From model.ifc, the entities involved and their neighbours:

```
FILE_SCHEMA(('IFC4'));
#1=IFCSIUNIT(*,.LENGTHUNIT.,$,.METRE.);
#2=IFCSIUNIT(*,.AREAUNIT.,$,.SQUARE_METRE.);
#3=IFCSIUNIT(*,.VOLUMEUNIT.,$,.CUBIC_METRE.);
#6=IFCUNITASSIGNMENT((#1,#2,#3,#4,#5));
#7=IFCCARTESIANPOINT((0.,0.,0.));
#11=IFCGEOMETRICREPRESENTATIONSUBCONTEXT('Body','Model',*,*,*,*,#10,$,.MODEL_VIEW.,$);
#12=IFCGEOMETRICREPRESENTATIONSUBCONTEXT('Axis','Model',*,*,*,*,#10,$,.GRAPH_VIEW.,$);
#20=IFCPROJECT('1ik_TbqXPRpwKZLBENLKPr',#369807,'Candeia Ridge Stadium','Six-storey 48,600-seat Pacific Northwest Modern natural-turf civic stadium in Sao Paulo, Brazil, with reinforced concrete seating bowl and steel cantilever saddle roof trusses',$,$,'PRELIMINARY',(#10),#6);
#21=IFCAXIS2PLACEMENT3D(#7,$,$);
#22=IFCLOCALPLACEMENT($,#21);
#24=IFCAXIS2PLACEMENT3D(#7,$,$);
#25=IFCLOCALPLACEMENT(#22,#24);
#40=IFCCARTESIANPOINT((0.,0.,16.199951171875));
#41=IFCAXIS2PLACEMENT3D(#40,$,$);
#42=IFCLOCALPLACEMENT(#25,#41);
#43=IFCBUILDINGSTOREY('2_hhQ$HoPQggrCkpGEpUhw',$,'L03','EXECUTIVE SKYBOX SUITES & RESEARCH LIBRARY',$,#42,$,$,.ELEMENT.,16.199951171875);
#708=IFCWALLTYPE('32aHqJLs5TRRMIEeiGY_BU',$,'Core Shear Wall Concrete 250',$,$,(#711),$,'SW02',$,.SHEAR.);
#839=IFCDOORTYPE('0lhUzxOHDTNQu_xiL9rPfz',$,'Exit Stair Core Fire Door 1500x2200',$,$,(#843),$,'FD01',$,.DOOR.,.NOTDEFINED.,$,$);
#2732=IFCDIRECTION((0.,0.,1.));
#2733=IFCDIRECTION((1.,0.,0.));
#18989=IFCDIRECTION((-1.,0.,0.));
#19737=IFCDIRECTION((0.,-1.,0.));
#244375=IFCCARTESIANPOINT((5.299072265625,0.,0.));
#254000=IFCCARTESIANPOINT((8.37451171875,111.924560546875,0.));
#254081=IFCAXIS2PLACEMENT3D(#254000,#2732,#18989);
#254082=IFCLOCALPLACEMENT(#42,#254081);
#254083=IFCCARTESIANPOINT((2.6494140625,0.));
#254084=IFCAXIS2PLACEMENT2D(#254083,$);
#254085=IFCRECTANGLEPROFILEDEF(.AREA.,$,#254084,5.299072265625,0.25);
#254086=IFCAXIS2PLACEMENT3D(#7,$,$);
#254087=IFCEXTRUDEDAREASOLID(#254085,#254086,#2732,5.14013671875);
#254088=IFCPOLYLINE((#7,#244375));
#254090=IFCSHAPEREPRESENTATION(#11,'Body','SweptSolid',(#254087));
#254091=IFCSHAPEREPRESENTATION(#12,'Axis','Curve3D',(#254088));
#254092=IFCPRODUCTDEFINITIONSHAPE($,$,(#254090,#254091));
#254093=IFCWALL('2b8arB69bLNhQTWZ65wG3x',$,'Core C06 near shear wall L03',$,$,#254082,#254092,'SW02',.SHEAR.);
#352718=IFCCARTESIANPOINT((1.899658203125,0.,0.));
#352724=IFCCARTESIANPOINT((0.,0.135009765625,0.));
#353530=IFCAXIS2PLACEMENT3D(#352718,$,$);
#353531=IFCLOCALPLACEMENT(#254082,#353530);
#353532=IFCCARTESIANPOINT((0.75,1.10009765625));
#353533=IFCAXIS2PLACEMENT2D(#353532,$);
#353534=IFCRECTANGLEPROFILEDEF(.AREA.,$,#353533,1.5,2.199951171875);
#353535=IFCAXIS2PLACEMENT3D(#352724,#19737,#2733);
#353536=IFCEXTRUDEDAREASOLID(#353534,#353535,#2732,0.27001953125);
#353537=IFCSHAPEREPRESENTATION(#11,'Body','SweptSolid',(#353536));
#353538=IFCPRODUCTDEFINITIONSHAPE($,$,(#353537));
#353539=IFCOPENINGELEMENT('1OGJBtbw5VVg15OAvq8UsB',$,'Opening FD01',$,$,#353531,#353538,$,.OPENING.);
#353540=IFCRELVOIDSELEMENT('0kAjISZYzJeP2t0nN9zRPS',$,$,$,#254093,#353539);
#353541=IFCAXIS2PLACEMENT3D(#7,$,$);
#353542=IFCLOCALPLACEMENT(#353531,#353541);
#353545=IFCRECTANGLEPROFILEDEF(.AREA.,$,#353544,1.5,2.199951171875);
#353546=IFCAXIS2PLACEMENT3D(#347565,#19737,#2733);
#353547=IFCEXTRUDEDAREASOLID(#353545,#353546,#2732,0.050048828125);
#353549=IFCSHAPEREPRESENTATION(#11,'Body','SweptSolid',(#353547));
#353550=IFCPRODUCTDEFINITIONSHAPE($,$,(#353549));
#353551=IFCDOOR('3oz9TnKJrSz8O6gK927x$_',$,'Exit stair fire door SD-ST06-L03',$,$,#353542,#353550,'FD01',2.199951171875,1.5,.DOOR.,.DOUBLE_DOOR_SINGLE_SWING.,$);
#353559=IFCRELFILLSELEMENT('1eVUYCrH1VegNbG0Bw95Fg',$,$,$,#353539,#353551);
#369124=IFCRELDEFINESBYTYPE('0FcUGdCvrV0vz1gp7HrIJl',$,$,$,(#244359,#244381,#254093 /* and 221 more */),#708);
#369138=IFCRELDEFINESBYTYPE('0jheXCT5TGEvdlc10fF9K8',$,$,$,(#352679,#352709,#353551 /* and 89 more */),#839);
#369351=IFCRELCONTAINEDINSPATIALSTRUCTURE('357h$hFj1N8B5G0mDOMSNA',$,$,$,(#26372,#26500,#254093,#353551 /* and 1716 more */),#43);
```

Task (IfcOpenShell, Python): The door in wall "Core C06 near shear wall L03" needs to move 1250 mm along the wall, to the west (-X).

```python
import ifcopenshell
import ifcopenshell.api.geometry
import ifcopenshell.util.placement

model = ifcopenshell.open("model.ifc")

door = model.by_id(353551)
opening = door.FillsVoids[0].RelatingOpeningElement
wall = opening.VoidsElements[0].RelatingBuildingElement

wall_matrix = ifcopenshell.util.placement.get_local_placement(wall.ObjectPlacement)
shift = wall_matrix[:3, 0] * 1.25
before = ifcopenshell.util.placement.get_local_placement(door.ObjectPlacement)[:3, 3].copy()

# The door is placed relative to its opening, so it follows when the opening moves.
matrix = ifcopenshell.util.placement.get_local_placement(opening.ObjectPlacement)
matrix[:3, 3] += shift
ifcopenshell.api.geometry.edit_object_placement(
    model, product=opening, matrix=matrix, is_si=False, should_transform_children=True
)

after = ifcopenshell.util.placement.get_local_placement(door.ObjectPlacement)[:3, 3]
print("door moved by", (after - before).round(3) + 0.0)

model.write("model_v2.ifc")
```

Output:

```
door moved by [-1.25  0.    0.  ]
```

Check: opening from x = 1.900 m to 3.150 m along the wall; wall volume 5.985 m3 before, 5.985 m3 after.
